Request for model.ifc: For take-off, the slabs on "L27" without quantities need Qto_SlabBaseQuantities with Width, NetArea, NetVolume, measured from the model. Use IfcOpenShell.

First a look at what the model holds.

```python
import ifcopenshell
import ifcopenshell.util.element
import ifcopenshell.util.unit

model = ifcopenshell.open("model.ifc")
print(model.schema)
for unit_type in ("LENGTHUNIT", "AREAUNIT", "VOLUMEUNIT"):
    print(unit_type, ifcopenshell.util.unit.calculate_unit_scale(model, unit_type))
storey = next(s for s in model.by_type("IfcBuildingStorey") if s.Name == "L27")
slabs = [e for e in ifcopenshell.util.element.get_decomposition(storey) if e.is_a("IfcSlab")]
for e in sorted(slabs, key=lambda e: e.id()):
    print(e.id(), e.is_a(), e.Name, list(ifcopenshell.util.element.get_psets(e, qtos_only=True)), sep=" | ")
```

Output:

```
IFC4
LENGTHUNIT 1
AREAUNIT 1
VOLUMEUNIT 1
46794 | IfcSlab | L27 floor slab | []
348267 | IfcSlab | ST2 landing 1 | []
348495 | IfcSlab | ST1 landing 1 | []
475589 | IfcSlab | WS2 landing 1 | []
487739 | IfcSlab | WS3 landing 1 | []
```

```python
import ifcopenshell
import ifcopenshell.api.pset
import ifcopenshell.geom
import ifcopenshell.util.element
import ifcopenshell.util.shape
import ifcopenshell.util.unit

model = ifcopenshell.open("model.ifc")
unit_scale = ifcopenshell.util.unit.calculate_unit_scale(model)
area_scale = ifcopenshell.util.unit.calculate_unit_scale(model, "AREAUNIT")
volume_scale = ifcopenshell.util.unit.calculate_unit_scale(model, "VOLUMEUNIT")
settings = ifcopenshell.geom.settings()

storey = next(s for s in model.by_type("IfcBuildingStorey") if s.Name == "L27")
slabs = [e for e in ifcopenshell.util.element.get_decomposition(storey) if e.is_a("IfcSlab")]

for e in sorted(slabs, key=lambda e: e.id()):
    if ifcopenshell.util.element.get_psets(e, qtos_only=True, should_inherit=False):
        continue
    # Geometry comes back in metres, in the element's own axes.
    shape = ifcopenshell.geom.create_shape(settings, e)
    values = {
        "Width": ifcopenshell.util.shape.get_z(shape.geometry) / unit_scale,
        "NetArea": ifcopenshell.util.shape.get_footprint_area(shape.geometry) / area_scale,
        "NetVolume": ifcopenshell.util.shape.get_volume(shape.geometry) / volume_scale,
    }
    qto = ifcopenshell.api.pset.add_qto(model, product=e, name="Qto_SlabBaseQuantities")
    ifcopenshell.api.pset.edit_qto(model, qto=qto, properties=values)
    print(e.id(), {k: round(v, 3) for k, v in values.items()})

model.write("model-out.ifc")
```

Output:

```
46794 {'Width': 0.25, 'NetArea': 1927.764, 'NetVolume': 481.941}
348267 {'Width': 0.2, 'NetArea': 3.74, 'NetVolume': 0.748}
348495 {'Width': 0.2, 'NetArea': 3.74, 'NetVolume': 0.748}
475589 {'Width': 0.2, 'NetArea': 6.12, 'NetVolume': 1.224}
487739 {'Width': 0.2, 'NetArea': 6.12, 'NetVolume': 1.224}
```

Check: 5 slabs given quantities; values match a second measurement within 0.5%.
